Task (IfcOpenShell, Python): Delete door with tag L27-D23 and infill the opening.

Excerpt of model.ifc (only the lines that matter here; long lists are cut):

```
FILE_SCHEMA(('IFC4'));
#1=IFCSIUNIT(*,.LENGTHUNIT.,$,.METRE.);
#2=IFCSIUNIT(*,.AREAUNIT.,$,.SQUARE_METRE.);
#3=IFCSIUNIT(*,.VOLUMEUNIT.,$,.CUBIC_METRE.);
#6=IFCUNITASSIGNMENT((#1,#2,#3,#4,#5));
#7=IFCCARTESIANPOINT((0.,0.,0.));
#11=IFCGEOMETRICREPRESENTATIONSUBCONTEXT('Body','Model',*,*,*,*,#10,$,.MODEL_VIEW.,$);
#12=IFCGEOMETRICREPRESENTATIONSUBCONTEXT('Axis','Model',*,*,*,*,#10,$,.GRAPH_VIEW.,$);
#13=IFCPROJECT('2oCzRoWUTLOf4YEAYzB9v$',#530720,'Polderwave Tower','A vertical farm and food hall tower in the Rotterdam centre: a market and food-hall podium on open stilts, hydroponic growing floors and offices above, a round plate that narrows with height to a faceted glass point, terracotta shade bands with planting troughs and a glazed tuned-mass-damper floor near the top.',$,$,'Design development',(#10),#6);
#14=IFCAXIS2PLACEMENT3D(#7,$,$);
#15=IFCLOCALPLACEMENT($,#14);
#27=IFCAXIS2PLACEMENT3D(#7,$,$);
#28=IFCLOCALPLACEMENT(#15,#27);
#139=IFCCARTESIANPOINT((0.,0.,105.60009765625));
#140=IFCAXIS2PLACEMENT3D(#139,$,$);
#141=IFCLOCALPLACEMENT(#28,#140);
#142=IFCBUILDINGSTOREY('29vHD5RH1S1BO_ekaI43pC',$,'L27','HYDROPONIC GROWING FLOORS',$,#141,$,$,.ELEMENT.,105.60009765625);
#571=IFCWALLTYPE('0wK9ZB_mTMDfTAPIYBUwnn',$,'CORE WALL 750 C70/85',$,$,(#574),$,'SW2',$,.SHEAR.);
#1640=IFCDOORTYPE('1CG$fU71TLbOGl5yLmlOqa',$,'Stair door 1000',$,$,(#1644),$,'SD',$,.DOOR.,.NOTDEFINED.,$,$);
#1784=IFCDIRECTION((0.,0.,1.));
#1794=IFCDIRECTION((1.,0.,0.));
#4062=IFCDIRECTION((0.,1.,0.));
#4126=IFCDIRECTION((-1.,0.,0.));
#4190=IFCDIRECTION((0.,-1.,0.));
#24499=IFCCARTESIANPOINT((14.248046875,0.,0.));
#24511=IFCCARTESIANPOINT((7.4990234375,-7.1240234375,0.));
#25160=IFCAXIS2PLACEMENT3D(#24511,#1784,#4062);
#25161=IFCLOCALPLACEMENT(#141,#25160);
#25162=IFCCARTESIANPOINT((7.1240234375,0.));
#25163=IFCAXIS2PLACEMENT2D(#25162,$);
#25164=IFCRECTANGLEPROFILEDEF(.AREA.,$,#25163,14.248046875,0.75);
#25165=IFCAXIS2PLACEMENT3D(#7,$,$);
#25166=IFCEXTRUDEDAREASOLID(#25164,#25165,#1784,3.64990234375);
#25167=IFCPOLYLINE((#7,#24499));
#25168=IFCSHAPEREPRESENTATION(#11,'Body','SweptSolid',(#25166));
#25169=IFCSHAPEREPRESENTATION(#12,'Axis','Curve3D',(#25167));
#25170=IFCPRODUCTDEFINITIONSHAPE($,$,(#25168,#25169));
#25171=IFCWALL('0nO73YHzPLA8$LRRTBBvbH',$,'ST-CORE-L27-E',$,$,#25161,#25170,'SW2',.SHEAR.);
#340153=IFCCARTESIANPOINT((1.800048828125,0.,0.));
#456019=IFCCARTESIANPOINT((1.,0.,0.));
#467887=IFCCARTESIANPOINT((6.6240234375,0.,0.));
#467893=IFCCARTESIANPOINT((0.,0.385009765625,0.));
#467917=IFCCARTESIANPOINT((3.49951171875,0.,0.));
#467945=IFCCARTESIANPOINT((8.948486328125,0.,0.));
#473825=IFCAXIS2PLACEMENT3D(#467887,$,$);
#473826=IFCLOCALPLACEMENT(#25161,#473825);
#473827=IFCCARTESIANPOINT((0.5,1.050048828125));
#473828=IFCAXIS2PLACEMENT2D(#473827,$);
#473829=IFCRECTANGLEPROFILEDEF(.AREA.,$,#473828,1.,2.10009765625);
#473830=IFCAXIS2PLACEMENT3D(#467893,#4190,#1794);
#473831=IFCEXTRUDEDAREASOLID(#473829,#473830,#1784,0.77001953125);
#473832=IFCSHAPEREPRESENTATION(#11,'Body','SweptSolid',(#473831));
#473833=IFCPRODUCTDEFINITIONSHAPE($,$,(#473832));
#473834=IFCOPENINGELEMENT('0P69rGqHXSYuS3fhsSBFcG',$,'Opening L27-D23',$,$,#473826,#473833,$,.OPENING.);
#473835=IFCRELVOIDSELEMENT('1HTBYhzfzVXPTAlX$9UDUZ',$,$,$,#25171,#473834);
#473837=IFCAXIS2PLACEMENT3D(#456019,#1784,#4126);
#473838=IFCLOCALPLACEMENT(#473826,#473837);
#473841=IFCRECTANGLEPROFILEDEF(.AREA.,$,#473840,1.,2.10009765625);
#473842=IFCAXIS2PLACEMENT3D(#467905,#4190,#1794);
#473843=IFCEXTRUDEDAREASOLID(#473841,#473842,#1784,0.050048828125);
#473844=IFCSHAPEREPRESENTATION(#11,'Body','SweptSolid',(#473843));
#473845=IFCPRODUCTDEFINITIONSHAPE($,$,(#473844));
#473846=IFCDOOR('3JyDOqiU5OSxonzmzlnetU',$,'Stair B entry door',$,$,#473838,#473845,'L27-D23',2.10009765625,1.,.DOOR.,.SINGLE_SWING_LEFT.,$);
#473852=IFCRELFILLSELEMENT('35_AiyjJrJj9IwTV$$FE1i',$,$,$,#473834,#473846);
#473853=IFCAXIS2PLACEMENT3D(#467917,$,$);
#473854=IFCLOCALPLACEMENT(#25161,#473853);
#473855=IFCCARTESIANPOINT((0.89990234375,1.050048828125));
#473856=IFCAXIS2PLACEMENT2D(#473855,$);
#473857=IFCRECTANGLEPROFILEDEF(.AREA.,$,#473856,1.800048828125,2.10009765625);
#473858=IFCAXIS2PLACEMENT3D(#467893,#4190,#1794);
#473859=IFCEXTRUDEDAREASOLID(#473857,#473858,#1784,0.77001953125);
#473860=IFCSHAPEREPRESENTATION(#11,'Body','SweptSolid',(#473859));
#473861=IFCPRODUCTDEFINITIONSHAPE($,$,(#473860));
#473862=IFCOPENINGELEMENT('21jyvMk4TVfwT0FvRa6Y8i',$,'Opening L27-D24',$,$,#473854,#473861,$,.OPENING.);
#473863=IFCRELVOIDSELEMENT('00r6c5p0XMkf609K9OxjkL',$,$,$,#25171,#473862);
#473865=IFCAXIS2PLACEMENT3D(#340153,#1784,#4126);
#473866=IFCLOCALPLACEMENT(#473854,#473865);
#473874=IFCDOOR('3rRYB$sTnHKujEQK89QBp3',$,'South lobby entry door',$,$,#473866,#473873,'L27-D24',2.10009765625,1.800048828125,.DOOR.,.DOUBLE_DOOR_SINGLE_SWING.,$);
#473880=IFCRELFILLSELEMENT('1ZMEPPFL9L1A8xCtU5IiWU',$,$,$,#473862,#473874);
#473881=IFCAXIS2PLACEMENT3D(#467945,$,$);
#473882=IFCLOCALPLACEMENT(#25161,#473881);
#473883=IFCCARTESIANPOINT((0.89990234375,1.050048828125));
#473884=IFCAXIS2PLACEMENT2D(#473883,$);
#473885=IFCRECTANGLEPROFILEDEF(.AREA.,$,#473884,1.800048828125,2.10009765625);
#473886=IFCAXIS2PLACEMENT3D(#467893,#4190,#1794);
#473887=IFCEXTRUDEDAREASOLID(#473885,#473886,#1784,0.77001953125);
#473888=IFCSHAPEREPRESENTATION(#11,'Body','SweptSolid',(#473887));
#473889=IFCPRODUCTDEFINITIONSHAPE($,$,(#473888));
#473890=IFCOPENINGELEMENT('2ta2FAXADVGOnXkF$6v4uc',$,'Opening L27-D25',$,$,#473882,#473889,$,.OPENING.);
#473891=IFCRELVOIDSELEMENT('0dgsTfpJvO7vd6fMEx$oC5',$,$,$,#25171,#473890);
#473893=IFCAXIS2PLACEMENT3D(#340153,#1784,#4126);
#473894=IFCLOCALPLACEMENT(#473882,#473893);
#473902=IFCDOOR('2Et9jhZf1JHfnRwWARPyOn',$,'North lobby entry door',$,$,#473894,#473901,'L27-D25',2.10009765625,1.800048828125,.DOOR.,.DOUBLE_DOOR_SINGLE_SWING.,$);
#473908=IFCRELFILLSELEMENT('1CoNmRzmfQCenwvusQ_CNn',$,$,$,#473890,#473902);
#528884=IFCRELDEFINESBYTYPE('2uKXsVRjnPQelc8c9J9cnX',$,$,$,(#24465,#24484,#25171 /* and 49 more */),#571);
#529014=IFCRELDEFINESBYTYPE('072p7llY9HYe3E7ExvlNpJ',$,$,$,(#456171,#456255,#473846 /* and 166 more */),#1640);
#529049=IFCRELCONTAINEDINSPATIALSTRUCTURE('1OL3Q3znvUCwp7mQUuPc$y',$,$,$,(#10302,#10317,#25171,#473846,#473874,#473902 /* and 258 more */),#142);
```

```python
import ifcopenshell
import ifcopenshell.api.feature
import ifcopenshell.api.root
import ifcopenshell.geom
import ifcopenshell.util.shape

model = ifcopenshell.open("model.ifc")
settings = ifcopenshell.geom.settings()


def volume(element):
    """Net volume in cubic metres, openings subtracted."""
    shape = ifcopenshell.geom.create_shape(settings, element)
    return ifcopenshell.util.shape.get_volume(shape.geometry)


door = model.by_guid("3JyDOqiU5OSxonzmzlnetU")
opening = door.FillsVoids[0].RelatingOpeningElement
wall = opening.VoidsElements[0].RelatingBuildingElement
before = volume(wall)

ifcopenshell.api.root.remove_product(model, product=door)
ifcopenshell.api.feature.remove_feature(model, feature=opening)

after = volume(wall)

print(f"wall volume {before:.3f} -> {after:.3f} m3")

model.write("model_edited.ifc")
```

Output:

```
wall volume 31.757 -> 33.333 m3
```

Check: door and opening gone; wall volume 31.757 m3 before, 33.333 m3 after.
